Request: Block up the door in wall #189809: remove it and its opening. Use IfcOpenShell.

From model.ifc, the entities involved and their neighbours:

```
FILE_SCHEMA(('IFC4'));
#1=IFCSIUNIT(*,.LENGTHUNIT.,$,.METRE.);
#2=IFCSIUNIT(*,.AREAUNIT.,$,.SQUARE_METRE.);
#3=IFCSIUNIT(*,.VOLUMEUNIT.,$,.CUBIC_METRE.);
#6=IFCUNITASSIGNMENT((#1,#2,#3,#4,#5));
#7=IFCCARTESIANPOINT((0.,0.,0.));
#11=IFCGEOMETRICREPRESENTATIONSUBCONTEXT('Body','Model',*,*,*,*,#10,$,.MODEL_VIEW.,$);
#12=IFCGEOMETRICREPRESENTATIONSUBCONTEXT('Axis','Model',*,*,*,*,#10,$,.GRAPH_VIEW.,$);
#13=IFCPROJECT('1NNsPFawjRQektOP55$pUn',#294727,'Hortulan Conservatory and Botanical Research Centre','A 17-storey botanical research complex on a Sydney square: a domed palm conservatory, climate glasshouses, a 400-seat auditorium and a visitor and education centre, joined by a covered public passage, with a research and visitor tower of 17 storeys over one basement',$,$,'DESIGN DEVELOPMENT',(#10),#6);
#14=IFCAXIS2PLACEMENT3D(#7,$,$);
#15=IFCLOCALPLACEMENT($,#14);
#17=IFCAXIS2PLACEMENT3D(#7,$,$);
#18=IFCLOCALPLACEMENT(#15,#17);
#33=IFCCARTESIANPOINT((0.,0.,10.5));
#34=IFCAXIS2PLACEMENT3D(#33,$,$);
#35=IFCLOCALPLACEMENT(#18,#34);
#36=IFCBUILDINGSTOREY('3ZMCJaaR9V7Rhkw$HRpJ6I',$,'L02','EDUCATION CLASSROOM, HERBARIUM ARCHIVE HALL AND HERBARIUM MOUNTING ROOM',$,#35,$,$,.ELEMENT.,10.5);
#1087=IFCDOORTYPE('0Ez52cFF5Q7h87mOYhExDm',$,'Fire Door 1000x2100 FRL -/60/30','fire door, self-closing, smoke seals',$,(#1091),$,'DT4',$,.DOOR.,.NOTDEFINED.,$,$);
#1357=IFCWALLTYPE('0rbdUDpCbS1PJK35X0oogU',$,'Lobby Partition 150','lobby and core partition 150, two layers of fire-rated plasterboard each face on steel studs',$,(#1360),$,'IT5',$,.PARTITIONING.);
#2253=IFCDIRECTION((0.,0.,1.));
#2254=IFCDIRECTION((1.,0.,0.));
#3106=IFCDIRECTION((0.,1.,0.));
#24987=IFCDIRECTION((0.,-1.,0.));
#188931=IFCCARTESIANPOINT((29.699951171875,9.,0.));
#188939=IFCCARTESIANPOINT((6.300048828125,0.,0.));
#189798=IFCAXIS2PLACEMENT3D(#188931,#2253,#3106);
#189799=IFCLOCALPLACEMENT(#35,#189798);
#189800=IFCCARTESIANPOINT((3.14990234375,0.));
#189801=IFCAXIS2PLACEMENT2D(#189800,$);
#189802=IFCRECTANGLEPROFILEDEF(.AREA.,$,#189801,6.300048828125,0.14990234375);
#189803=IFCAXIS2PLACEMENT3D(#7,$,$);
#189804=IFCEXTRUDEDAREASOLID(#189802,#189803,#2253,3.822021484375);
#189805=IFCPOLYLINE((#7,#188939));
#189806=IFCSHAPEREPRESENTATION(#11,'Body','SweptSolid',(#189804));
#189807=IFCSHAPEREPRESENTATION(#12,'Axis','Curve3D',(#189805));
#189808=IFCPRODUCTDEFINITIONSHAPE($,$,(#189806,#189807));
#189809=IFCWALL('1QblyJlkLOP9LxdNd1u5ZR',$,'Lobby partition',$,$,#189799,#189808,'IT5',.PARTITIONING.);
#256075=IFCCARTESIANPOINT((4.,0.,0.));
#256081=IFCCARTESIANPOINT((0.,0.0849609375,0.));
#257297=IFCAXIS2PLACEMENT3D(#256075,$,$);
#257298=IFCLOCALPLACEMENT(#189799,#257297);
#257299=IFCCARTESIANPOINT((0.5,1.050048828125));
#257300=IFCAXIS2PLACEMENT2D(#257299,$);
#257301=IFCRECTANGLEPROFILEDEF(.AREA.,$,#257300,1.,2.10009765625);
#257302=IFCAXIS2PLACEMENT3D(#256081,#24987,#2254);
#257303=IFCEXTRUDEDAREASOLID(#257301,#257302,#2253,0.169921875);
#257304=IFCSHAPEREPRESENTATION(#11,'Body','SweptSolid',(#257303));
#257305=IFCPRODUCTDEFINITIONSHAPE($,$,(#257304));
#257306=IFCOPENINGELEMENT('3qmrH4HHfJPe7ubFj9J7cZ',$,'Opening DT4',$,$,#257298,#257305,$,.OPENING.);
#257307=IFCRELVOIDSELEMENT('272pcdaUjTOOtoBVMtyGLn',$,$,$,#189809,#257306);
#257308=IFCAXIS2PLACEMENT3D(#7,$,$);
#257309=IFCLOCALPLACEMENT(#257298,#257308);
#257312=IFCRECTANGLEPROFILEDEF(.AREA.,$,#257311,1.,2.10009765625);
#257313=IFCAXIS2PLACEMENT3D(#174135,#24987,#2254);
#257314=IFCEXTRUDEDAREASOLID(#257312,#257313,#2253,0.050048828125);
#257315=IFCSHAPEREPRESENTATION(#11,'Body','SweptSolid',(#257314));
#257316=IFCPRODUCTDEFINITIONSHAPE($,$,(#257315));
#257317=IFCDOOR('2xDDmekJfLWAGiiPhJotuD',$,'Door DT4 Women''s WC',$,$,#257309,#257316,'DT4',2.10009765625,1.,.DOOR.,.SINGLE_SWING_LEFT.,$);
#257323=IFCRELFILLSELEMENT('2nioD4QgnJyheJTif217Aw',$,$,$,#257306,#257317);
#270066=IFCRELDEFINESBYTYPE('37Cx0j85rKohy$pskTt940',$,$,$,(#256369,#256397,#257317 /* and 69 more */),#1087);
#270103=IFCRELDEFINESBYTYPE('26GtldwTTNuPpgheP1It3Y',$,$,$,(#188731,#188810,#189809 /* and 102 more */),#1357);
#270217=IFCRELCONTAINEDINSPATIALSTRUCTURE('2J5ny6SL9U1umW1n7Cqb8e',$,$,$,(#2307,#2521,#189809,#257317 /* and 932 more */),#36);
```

```python
import ifcopenshell
import ifcopenshell.api.feature
import ifcopenshell.api.root
import ifcopenshell.geom
import ifcopenshell.util.shape

model = ifcopenshell.open("model.ifc")
settings = ifcopenshell.geom.settings()


def volume(element):
    """Net volume in cubic metres, openings subtracted."""
    shape = ifcopenshell.geom.create_shape(settings, element)
    return ifcopenshell.util.shape.get_volume(shape.geometry)


door = model.by_guid("2xDDmekJfLWAGiiPhJotuD")
opening = door.FillsVoids[0].RelatingOpeningElement
wall = opening.VoidsElements[0].RelatingBuildingElement
before = volume(wall)

ifcopenshell.api.root.remove_product(model, product=door)
ifcopenshell.api.feature.remove_feature(model, feature=opening)

after = volume(wall)

print(f"wall volume {before:.3f} -> {after:.3f} m3")

model.write("model_updated.ifc")
```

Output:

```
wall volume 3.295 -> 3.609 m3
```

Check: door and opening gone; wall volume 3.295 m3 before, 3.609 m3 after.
